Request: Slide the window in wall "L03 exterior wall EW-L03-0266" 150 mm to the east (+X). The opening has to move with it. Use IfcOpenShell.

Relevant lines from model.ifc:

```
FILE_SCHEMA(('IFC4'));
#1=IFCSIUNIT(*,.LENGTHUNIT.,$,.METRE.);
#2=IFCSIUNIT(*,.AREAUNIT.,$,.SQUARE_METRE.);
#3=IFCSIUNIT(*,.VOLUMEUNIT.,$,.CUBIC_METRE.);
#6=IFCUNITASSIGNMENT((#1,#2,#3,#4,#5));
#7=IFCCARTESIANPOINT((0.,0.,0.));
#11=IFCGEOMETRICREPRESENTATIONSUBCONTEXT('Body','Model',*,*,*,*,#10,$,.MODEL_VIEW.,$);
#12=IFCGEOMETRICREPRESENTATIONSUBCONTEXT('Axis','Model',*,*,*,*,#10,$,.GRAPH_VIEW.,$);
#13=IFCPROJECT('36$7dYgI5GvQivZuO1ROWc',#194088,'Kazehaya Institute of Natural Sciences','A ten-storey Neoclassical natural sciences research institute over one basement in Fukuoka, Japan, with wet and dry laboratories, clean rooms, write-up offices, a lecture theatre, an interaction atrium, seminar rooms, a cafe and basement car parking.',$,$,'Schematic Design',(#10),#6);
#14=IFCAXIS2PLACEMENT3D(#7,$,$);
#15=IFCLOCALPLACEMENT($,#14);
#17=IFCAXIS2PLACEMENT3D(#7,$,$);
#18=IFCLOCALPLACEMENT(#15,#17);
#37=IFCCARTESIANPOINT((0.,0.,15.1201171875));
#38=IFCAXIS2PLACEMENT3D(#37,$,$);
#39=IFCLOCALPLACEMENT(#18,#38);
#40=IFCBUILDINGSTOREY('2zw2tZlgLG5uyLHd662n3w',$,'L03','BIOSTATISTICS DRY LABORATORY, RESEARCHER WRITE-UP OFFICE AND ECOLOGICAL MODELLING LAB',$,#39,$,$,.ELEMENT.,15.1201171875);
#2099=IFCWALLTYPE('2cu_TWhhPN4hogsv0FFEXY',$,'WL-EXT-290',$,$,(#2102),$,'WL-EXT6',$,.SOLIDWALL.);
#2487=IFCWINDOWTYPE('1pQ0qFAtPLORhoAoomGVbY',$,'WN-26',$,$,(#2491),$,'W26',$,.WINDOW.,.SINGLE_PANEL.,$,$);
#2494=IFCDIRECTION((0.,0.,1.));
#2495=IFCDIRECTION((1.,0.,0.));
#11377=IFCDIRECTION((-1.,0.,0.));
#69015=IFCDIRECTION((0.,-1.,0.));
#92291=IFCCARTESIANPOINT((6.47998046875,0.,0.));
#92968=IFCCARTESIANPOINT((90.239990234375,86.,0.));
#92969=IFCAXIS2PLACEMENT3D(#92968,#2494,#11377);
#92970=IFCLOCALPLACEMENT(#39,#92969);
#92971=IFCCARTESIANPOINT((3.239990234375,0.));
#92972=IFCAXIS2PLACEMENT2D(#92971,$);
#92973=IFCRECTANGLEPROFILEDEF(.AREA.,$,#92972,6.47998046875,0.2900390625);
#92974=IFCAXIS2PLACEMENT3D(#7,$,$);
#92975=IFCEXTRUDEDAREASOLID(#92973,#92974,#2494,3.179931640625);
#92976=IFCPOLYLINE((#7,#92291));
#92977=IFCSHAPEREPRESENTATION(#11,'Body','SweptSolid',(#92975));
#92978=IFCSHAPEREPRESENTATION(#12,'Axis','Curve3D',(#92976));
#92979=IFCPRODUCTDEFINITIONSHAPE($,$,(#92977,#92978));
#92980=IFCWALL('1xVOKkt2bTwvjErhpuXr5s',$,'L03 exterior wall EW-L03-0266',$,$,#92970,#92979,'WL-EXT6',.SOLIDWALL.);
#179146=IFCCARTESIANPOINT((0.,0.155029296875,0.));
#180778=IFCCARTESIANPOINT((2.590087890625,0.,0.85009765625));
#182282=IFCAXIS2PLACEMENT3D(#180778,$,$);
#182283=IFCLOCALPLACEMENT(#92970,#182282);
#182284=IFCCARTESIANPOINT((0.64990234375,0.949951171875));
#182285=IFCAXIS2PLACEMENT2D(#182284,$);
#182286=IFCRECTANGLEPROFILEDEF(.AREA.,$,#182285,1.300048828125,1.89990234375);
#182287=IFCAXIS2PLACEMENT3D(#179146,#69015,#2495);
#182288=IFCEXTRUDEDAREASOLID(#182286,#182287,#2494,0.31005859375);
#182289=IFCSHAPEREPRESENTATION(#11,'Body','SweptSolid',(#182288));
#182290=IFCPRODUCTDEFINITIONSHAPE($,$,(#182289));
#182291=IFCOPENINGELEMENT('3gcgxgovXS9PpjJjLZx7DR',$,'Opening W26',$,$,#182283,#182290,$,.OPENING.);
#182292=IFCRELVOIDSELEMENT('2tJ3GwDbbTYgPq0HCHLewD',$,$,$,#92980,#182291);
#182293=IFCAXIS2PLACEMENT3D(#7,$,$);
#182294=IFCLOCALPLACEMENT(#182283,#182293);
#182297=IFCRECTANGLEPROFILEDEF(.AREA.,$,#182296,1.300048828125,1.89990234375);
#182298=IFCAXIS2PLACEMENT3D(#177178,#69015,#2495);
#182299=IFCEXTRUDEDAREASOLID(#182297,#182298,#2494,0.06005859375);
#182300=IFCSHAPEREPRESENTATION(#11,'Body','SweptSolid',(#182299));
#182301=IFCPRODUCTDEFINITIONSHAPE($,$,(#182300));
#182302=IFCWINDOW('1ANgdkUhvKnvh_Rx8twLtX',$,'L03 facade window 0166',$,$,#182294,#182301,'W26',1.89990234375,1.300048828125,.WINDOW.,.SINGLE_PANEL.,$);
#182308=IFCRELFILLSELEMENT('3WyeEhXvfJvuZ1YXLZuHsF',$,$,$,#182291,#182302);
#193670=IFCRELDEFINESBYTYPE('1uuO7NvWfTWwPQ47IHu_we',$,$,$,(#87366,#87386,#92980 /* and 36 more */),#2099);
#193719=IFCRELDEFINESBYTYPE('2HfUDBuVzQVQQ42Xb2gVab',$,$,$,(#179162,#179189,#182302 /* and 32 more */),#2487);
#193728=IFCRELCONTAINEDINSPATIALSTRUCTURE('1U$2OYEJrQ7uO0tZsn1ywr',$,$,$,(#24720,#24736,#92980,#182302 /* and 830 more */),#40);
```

```python
import ifcopenshell
import ifcopenshell.api.geometry
import ifcopenshell.util.placement
import ifcopenshell.util.unit

model = ifcopenshell.open("model.ifc")
unit_scale = ifcopenshell.util.unit.calculate_unit_scale(model)

window = model.by_id(182302)
opening = window.FillsVoids[0].RelatingOpeningElement
wall = opening.VoidsElements[0].RelatingBuildingElement

wall_matrix = ifcopenshell.util.placement.get_local_placement(wall.ObjectPlacement)
shift = wall_matrix[:3, 0] * -0.15 / unit_scale
before = ifcopenshell.util.placement.get_local_placement(window.ObjectPlacement)[:3, 3].copy()

# The window is placed relative to its opening, so it follows when the opening moves.
matrix = ifcopenshell.util.placement.get_local_placement(opening.ObjectPlacement)
matrix[:3, 3] += shift
ifcopenshell.api.geometry.edit_object_placement(
    model, product=opening, matrix=matrix, is_si=False, should_transform_children=True
)

after = ifcopenshell.util.placement.get_local_placement(window.ObjectPlacement)[:3, 3]
print("window moved by", (after - before).round(3) + 0.0)

model.write("model_updated.ifc")
```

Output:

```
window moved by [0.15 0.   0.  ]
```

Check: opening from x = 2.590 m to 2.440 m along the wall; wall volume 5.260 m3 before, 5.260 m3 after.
